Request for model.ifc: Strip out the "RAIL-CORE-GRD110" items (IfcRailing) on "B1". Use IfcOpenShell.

First a look at what the model holds.

```python
import ifcopenshell
import ifcopenshell.util.element

model = ifcopenshell.open("model.ifc")
print(model.schema)
storey = next(s for s in model.by_type("IfcBuildingStorey") if s.Name == "B1")
railings = [e for e in ifcopenshell.util.element.get_decomposition(storey) if e.is_a("IfcRailing")]
seen = {}
for e in railings:
    element_type = ifcopenshell.util.element.get_type(e)
    name = element_type.Name if element_type not in (None, e) else None
    seen[name] = seen.get(name, 0) + 1
for name, count in sorted(seen.items(), key=str):
    print(count, "x", name)
```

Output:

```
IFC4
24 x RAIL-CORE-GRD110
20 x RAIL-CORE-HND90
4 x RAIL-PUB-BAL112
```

```python
import ifcopenshell
import ifcopenshell.api.root
import ifcopenshell.util.element

model = ifcopenshell.open("model.ifc")

storey = next(s for s in model.by_type("IfcBuildingStorey") if s.Name == "B1")
railings = [e for e in ifcopenshell.util.element.get_decomposition(storey) if e.is_a("IfcRailing")]
targets = [e for e in railings if (t := ifcopenshell.util.element.get_type(e)) not in (None, e) and t.Name == "RAIL-CORE-GRD110"]

for e in targets:
    ifcopenshell.api.root.remove_product(model, product=e)
print(len(targets), "removed")

model.write("model_v2.ifc")
```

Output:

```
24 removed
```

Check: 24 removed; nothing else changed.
